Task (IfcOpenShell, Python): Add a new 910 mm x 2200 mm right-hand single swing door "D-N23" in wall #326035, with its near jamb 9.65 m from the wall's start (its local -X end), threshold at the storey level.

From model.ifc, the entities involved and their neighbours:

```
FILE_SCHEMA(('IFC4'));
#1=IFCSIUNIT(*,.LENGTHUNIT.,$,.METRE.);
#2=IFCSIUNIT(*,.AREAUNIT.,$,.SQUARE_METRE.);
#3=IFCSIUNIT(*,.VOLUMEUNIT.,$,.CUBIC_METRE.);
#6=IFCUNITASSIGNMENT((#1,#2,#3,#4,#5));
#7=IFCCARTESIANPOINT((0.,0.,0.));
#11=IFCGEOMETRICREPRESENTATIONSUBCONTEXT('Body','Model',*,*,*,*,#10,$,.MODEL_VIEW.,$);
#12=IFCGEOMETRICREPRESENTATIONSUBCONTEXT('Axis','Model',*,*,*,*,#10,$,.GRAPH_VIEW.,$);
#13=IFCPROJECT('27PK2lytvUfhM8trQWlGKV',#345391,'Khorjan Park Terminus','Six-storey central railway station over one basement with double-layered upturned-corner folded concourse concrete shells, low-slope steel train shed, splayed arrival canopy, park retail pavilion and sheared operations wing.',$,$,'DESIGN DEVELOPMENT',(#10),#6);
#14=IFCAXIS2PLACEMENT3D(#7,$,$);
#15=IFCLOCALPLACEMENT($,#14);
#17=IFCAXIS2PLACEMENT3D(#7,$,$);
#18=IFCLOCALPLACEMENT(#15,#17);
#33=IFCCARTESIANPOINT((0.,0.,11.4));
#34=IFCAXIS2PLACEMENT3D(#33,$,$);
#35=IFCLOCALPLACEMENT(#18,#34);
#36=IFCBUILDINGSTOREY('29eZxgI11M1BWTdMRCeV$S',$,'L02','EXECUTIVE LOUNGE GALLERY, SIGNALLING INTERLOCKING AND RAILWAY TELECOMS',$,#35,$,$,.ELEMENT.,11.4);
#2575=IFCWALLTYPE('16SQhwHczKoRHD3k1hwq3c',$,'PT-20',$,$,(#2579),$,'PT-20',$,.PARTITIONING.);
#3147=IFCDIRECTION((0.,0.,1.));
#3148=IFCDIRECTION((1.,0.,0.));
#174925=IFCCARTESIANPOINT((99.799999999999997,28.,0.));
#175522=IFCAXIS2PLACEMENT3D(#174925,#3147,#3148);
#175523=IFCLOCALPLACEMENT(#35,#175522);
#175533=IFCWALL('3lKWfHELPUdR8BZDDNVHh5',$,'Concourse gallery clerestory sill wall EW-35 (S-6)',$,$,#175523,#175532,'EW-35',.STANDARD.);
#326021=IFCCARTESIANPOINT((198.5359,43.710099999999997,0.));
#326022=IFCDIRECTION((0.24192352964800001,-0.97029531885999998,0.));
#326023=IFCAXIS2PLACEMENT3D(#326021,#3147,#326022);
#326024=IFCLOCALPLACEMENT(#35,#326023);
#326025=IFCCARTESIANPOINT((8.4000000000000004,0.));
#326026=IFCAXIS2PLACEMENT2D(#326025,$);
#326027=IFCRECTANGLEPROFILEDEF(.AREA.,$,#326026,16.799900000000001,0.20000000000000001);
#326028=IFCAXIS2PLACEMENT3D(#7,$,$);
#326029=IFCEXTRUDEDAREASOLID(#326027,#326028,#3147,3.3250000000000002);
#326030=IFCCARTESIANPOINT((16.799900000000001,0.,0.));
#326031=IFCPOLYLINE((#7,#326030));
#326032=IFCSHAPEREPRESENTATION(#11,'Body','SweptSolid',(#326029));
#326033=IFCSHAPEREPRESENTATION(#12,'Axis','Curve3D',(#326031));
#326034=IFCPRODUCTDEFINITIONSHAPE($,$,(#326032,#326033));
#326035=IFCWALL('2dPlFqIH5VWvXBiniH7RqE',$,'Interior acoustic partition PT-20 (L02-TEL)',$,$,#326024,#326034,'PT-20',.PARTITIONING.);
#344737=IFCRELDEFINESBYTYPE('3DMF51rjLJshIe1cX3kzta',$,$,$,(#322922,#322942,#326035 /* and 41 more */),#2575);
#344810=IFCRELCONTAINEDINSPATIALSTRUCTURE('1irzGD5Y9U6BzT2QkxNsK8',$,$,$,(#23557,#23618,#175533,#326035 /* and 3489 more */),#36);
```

```python
import numpy as np
import ifcopenshell
import ifcopenshell.api.feature
import ifcopenshell.api.geometry
import ifcopenshell.api.root
import ifcopenshell.api.spatial
import ifcopenshell.geom
import ifcopenshell.util.element
import ifcopenshell.util.placement
import ifcopenshell.util.representation
import ifcopenshell.util.shape
import ifcopenshell.util.unit

model = ifcopenshell.open("model.ifc")
unit_scale = ifcopenshell.util.unit.calculate_unit_scale(model)
settings = ifcopenshell.geom.settings()


def volume(element):
    """Net volume in cubic metres, openings subtracted."""
    shape = ifcopenshell.geom.create_shape(settings, element)
    return ifcopenshell.util.shape.get_volume(shape.geometry)


wall = model.by_guid("2dPlFqIH5VWvXBiniH7RqE")
storey = ifcopenshell.util.element.get_container(wall, ifc_class="IfcBuildingStorey")
context = ifcopenshell.util.representation.get_context(model, "Model", "Body", "MODEL_VIEW")
before = volume(wall)

width, height, from_end, sill = 0.91, 2.2, 9.65, 0.0  # metres

# The wall runs along its own X axis, and the end named is its -X end.
wall_shape = ifcopenshell.geom.create_shape(settings, wall)
x, y, z = ifcopenshell.util.shape.get_vertices(wall_shape.geometry).T
start = x.min() + from_end
face, thickness = float(y.min()), float(y.max() - y.min())
wall_matrix = ifcopenshell.util.placement.get_local_placement(wall.ObjectPlacement)
level = ifcopenshell.util.placement.get_local_placement(storey.ObjectPlacement)[2, 3]


def in_wall(x, y):
    """Placement at x, y metres in the wall's axes, at sill height."""
    matrix = wall_matrix.copy()
    matrix[:, 3] = wall_matrix @ np.array([x / unit_scale, y / unit_scale, 0.0, 1.0])
    matrix[2, 3] = level + sill / unit_scale
    return matrix


# Opening: a box that overshoots both wall faces by 50 mm.
opening = ifcopenshell.api.root.create_entity(model, ifc_class="IfcOpeningElement", predefined_type="OPENING")
box = ifcopenshell.api.geometry.add_wall_representation(
    model, context=context, length=width, height=height, thickness=thickness + 0.1
)
ifcopenshell.api.geometry.assign_representation(model, product=opening, representation=box)
ifcopenshell.api.geometry.edit_object_placement(model, product=opening, matrix=in_wall(start, face - 0.05), is_si=False)
ifcopenshell.api.feature.add_feature(model, feature=opening, element=wall)

door = ifcopenshell.api.root.create_entity(model, ifc_class="IfcDoor", name="D-N23", predefined_type="DOOR")
door.OverallWidth, door.OverallHeight = width / unit_scale, height / unit_scale
door.OperationType = "SINGLE_SWING_RIGHT"
body = ifcopenshell.api.geometry.add_door_representation(
    model,
    context=context,
    overall_width=door.OverallWidth,
    overall_height=door.OverallHeight,
    operation_type="SINGLE_SWING_RIGHT",
    lining_properties={"LiningDepth": thickness / unit_scale, "ThresholdDepth": thickness / unit_scale},
)
ifcopenshell.api.geometry.assign_representation(model, product=door, representation=body)
ifcopenshell.api.spatial.assign_container(model, products=[door], relating_structure=storey)
ifcopenshell.api.feature.add_filling(model, opening=opening, element=door)

# The lining spans the wall, so the door starts at the wall face.
ifcopenshell.api.geometry.edit_object_placement(model, product=door, matrix=in_wall(start, face), is_si=False)

after = volume(wall)

print(f"wall volume {before:.3f} -> {after:.3f} m3")

model.write("model_edited.ifc")
```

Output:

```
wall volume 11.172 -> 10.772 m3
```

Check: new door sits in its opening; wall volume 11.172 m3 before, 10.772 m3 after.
